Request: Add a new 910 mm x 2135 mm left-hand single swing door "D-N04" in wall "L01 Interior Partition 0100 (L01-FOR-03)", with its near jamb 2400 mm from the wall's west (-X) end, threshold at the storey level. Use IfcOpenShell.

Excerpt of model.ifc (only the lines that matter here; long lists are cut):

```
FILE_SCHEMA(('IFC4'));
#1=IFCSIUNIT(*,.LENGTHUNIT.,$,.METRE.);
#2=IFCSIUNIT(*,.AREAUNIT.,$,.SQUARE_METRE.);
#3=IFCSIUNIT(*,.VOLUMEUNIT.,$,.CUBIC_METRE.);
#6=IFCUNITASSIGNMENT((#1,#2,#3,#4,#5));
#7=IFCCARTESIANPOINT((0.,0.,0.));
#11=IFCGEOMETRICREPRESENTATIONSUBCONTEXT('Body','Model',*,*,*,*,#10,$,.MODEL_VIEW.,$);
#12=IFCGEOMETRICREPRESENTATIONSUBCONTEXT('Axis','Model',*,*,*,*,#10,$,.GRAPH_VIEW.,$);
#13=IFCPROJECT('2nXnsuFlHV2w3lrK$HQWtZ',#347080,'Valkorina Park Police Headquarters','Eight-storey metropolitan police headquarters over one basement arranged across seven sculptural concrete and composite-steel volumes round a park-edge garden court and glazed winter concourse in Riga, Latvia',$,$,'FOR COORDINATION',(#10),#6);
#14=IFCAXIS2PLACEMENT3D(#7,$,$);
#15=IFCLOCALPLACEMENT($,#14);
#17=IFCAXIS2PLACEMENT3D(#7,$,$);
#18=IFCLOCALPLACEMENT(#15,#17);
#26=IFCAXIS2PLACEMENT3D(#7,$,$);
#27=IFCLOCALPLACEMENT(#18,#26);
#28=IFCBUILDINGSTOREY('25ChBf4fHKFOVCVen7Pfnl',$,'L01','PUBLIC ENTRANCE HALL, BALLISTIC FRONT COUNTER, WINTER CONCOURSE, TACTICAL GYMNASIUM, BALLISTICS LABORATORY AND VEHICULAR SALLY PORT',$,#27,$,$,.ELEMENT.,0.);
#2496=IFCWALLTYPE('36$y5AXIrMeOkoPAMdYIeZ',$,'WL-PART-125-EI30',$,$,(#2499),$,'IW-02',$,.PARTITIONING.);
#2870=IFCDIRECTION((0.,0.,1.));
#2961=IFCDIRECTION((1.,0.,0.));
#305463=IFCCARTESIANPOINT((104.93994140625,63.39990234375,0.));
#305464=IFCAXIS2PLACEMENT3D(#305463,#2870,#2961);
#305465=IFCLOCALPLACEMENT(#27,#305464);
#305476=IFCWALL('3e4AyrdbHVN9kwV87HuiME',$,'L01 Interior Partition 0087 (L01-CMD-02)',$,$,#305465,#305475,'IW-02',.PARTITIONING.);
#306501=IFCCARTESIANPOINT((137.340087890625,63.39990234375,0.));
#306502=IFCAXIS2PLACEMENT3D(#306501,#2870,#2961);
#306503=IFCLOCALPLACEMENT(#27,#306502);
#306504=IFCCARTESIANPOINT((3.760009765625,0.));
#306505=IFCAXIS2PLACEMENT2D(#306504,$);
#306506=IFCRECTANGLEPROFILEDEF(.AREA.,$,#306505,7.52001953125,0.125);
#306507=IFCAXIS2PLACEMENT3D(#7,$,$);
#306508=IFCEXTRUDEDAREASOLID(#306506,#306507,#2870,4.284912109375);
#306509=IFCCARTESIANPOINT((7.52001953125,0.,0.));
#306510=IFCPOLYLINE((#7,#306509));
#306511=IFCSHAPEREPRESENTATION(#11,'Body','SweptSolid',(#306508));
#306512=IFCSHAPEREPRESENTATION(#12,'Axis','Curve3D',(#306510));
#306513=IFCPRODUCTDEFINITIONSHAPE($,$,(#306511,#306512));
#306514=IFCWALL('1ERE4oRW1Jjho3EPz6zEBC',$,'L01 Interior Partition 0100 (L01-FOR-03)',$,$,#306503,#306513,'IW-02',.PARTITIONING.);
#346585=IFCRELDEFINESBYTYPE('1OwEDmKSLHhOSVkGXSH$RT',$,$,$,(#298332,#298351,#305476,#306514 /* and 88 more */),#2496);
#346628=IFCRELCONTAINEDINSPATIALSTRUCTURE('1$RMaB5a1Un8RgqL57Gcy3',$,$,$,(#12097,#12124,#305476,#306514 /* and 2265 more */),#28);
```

```python
import numpy as np
import ifcopenshell
import ifcopenshell.api.feature
import ifcopenshell.api.geometry
import ifcopenshell.api.root
import ifcopenshell.api.spatial
import ifcopenshell.geom
import ifcopenshell.util.element
import ifcopenshell.util.placement
import ifcopenshell.util.representation
import ifcopenshell.util.shape
import ifcopenshell.util.unit

model = ifcopenshell.open("model.ifc")
unit_scale = ifcopenshell.util.unit.calculate_unit_scale(model)
settings = ifcopenshell.geom.settings()


def volume(element):
    """Net volume in cubic metres, openings subtracted."""
    shape = ifcopenshell.geom.create_shape(settings, element)
    return ifcopenshell.util.shape.get_volume(shape.geometry)


wall = model.by_id(306514)
storey = ifcopenshell.util.element.get_container(wall, ifc_class="IfcBuildingStorey")
context = ifcopenshell.util.representation.get_context(model, "Model", "Body", "MODEL_VIEW")
before = volume(wall)

width, height, from_end, sill = 0.91, 2.135, 2.4, 0.0  # metres

# The wall runs along its own X axis, and the end named is its -X end.
wall_shape = ifcopenshell.geom.create_shape(settings, wall)
x, y, z = ifcopenshell.util.shape.get_vertices(wall_shape.geometry).T
start = x.min() + from_end
face, thickness = float(y.min()), float(y.max() - y.min())
wall_matrix = ifcopenshell.util.placement.get_local_placement(wall.ObjectPlacement)
level = ifcopenshell.util.placement.get_local_placement(storey.ObjectPlacement)[2, 3]


def in_wall(x, y):
    """Placement at x, y metres in the wall's axes, at sill height."""
    matrix = wall_matrix.copy()
    matrix[:, 3] = wall_matrix @ np.array([x / unit_scale, y / unit_scale, 0.0, 1.0])
    matrix[2, 3] = level + sill / unit_scale
    return matrix


# Opening: a box that overshoots both wall faces by 50 mm.
opening = ifcopenshell.api.root.create_entity(model, ifc_class="IfcOpeningElement", predefined_type="OPENING")
box = ifcopenshell.api.geometry.add_wall_representation(
    model, context=context, length=width, height=height, thickness=thickness + 0.1
)
ifcopenshell.api.geometry.assign_representation(model, product=opening, representation=box)
ifcopenshell.api.geometry.edit_object_placement(model, product=opening, matrix=in_wall(start, face - 0.05), is_si=False)
ifcopenshell.api.feature.add_feature(model, feature=opening, element=wall)

door = ifcopenshell.api.root.create_entity(model, ifc_class="IfcDoor", name="D-N04", predefined_type="DOOR")
door.OverallWidth, door.OverallHeight = width / unit_scale, height / unit_scale
door.OperationType = "SINGLE_SWING_LEFT"
body = ifcopenshell.api.geometry.add_door_representation(
    model,
    context=context,
    overall_width=door.OverallWidth,
    overall_height=door.OverallHeight,
    operation_type="SINGLE_SWING_LEFT",
    lining_properties={"LiningDepth": thickness / unit_scale, "ThresholdDepth": thickness / unit_scale},
)
ifcopenshell.api.geometry.assign_representation(model, product=door, representation=body)
ifcopenshell.api.spatial.assign_container(model, products=[door], relating_structure=storey)
ifcopenshell.api.feature.add_filling(model, opening=opening, element=door)

# The lining spans the wall, so the door starts at the wall face.
ifcopenshell.api.geometry.edit_object_placement(model, product=door, matrix=in_wall(start, face), is_si=False)

after = volume(wall)

print(f"wall volume {before:.3f} -> {after:.3f} m3")

model.write("model_v2.ifc")
```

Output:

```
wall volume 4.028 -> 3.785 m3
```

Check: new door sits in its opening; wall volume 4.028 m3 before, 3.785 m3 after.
